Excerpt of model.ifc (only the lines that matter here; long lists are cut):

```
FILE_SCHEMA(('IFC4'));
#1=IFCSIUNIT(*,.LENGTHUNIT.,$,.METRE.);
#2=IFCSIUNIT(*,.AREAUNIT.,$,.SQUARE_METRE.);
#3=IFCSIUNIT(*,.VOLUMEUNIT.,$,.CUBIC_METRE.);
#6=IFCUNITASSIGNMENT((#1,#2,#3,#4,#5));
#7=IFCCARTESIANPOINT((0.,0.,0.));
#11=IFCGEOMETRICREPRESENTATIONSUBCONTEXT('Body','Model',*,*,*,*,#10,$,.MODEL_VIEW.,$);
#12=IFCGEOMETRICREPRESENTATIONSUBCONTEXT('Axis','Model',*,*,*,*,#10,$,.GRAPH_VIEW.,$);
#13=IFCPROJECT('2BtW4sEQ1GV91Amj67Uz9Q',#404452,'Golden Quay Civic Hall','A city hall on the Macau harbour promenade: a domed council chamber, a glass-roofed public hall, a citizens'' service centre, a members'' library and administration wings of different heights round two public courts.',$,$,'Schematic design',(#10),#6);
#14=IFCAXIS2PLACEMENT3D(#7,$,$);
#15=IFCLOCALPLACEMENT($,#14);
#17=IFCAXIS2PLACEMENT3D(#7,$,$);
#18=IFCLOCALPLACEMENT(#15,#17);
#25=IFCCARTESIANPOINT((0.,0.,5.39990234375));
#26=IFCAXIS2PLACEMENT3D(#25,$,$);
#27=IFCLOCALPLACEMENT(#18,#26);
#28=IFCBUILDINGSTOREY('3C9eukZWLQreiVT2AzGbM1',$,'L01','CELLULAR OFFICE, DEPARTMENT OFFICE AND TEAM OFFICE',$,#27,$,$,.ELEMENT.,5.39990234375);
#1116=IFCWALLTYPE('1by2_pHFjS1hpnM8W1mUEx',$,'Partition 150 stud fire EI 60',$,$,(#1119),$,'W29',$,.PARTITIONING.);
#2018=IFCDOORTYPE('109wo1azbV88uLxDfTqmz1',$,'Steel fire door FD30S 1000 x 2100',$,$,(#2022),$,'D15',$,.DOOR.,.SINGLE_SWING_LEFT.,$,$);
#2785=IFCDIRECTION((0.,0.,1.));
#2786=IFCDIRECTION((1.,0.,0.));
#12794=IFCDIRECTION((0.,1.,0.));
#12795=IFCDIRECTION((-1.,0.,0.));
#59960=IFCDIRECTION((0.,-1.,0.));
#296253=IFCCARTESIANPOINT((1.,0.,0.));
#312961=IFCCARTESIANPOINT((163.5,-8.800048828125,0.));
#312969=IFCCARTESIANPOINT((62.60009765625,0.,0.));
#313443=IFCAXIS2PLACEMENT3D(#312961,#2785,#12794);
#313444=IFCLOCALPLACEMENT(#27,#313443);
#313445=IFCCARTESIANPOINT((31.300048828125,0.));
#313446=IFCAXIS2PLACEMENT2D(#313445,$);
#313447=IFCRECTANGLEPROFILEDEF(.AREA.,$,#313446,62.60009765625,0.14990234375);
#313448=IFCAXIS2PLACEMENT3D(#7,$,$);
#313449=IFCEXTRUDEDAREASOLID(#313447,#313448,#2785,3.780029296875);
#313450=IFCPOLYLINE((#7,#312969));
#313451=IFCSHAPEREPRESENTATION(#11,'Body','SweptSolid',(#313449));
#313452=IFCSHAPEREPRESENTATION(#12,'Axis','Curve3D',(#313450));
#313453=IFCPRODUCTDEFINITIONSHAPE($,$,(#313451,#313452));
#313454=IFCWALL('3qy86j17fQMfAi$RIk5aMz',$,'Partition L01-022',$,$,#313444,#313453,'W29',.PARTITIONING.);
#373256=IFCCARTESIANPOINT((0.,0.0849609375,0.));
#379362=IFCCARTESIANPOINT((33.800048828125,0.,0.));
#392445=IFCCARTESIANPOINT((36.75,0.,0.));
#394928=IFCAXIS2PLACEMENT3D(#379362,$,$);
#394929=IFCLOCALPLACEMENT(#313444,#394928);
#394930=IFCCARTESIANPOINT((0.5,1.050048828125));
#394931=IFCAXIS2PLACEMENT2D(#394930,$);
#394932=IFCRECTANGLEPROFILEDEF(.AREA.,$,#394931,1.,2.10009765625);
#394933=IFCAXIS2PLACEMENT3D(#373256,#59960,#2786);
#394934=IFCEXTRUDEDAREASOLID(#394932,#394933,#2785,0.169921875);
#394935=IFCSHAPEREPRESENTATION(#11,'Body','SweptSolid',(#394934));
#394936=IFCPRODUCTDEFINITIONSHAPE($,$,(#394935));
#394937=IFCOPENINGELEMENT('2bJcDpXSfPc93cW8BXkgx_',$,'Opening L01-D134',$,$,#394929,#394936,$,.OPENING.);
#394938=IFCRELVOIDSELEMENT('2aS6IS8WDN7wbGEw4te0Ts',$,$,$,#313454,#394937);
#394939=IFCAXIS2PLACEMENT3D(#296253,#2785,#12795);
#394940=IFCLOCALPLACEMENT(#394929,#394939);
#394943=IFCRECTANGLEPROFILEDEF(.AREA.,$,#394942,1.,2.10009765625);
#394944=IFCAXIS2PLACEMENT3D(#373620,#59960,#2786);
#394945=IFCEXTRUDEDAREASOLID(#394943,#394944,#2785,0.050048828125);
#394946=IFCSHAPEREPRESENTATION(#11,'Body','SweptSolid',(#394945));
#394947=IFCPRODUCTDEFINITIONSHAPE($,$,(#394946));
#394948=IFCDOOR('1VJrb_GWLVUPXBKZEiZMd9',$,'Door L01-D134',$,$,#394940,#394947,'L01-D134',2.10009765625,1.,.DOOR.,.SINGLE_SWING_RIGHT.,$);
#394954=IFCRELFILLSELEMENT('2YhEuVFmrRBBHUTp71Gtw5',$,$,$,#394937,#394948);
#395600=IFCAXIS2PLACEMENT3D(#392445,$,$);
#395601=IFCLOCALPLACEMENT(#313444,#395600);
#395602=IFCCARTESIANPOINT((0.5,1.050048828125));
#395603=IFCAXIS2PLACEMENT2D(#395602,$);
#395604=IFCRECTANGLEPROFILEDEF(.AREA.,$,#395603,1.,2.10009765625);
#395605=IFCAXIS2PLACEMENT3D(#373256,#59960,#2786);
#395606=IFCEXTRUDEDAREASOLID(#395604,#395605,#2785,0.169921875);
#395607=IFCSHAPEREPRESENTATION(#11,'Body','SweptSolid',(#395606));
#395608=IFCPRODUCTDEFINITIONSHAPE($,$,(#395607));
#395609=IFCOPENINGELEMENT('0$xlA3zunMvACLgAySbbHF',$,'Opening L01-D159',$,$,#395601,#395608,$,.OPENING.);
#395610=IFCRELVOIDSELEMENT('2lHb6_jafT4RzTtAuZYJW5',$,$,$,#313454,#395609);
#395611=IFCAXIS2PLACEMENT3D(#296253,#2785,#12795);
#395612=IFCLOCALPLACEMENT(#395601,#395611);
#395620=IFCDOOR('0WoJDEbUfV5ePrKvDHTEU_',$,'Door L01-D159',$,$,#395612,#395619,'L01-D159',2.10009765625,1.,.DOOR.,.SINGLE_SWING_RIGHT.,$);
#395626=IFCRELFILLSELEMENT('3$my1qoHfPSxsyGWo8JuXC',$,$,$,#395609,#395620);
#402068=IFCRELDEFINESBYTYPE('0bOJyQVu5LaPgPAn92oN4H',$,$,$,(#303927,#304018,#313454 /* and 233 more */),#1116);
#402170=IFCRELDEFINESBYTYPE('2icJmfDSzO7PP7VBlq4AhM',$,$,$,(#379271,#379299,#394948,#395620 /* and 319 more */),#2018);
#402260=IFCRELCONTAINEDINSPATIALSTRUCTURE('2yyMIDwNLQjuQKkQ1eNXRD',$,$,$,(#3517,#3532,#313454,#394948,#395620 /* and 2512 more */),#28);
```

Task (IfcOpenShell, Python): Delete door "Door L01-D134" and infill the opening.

```python
import ifcopenshell
import ifcopenshell.api.feature
import ifcopenshell.api.root
import ifcopenshell.geom
import ifcopenshell.util.shape

model = ifcopenshell.open("model.ifc")
settings = ifcopenshell.geom.settings()


def volume(element):
    """Net volume in cubic metres, openings subtracted."""
    shape = ifcopenshell.geom.create_shape(settings, element)
    return ifcopenshell.util.shape.get_volume(shape.geometry)


door = model.by_guid("1VJrb_GWLVUPXBKZEiZMd9")
opening = door.FillsVoids[0].RelatingOpeningElement
wall = opening.VoidsElements[0].RelatingBuildingElement
before = volume(wall)

ifcopenshell.api.root.remove_product(model, product=door)
ifcopenshell.api.feature.remove_feature(model, feature=opening)

after = volume(wall)

print(f"wall volume {before:.3f} -> {after:.3f} m3")

model.write("model-out.ifc")
```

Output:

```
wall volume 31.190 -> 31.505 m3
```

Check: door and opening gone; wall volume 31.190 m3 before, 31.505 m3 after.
